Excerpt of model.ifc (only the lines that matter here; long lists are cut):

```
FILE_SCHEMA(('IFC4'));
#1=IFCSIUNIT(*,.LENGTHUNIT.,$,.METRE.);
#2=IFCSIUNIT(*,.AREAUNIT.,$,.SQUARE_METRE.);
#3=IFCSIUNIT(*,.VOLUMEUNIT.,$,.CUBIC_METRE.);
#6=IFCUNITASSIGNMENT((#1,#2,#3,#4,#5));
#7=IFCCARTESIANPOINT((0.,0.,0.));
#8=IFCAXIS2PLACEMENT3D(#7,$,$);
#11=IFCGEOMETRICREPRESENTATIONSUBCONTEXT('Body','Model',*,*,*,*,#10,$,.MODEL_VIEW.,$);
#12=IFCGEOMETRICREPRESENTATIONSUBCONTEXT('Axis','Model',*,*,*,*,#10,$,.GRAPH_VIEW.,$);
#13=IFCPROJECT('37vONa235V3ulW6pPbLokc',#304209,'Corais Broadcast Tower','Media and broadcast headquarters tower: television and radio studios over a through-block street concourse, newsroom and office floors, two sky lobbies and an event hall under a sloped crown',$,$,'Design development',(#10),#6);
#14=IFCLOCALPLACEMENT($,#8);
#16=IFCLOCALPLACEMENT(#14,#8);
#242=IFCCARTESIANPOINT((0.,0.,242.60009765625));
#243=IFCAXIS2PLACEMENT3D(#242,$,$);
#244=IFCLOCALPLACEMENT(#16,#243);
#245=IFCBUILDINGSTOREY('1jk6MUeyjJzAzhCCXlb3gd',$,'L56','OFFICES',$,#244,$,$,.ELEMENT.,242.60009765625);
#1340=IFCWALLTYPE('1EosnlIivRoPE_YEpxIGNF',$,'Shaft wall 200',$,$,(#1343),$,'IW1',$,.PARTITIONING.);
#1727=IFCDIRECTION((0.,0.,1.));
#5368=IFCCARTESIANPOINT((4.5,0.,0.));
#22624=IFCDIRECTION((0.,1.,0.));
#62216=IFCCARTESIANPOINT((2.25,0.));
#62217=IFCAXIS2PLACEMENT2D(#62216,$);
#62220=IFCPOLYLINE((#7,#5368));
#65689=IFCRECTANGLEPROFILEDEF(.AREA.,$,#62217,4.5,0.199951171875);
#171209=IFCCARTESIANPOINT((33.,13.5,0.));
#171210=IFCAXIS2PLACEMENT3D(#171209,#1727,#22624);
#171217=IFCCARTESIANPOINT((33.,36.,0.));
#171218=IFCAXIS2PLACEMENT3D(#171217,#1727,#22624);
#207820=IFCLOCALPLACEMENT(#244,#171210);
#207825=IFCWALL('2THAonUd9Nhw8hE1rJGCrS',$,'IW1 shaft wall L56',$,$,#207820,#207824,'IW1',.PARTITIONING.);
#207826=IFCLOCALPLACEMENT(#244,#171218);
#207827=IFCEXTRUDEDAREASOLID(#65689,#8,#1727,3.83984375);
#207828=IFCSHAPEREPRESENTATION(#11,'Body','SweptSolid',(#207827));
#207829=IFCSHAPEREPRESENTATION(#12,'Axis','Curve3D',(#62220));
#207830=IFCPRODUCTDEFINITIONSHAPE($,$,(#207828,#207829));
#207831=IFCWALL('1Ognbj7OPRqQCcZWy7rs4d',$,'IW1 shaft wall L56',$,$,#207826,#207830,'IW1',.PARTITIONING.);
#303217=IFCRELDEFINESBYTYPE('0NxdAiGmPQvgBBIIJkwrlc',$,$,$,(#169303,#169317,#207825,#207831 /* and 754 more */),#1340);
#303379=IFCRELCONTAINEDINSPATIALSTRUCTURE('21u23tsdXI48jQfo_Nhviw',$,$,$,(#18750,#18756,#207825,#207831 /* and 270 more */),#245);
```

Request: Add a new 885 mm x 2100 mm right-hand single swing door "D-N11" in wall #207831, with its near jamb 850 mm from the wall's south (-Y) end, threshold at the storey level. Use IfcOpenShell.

```python
import numpy as np
import ifcopenshell
import ifcopenshell.api.feature
import ifcopenshell.api.geometry
import ifcopenshell.api.root
import ifcopenshell.api.spatial
import ifcopenshell.geom
import ifcopenshell.util.element
import ifcopenshell.util.placement
import ifcopenshell.util.representation
import ifcopenshell.util.shape
import ifcopenshell.util.unit

model = ifcopenshell.open("model.ifc")
unit_scale = ifcopenshell.util.unit.calculate_unit_scale(model)
settings = ifcopenshell.geom.settings()


def volume(element):
    """Net volume in cubic metres, openings subtracted."""
    shape = ifcopenshell.geom.create_shape(settings, element)
    return ifcopenshell.util.shape.get_volume(shape.geometry)


wall = model.by_guid("1Ognbj7OPRqQCcZWy7rs4d")
storey = ifcopenshell.util.element.get_container(wall, ifc_class="IfcBuildingStorey")
context = ifcopenshell.util.representation.get_context(model, "Model", "Body", "MODEL_VIEW")
before = volume(wall)

width, height, from_end, sill = 0.885, 2.1, 0.85, 0.0  # metres

# The wall runs along its own X axis, and the end named is its -X end.
wall_shape = ifcopenshell.geom.create_shape(settings, wall)
x, y, z = ifcopenshell.util.shape.get_vertices(wall_shape.geometry).T
start = x.min() + from_end
face, thickness = float(y.min()), float(y.max() - y.min())
wall_matrix = ifcopenshell.util.placement.get_local_placement(wall.ObjectPlacement)
level = ifcopenshell.util.placement.get_local_placement(storey.ObjectPlacement)[2, 3]


def in_wall(x, y):
    """Placement at x, y metres in the wall's axes, at sill height."""
    matrix = wall_matrix.copy()
    matrix[:, 3] = wall_matrix @ np.array([x / unit_scale, y / unit_scale, 0.0, 1.0])
    matrix[2, 3] = level + sill / unit_scale
    return matrix


# Opening: a box that overshoots both wall faces by 50 mm.
opening = ifcopenshell.api.root.create_entity(model, ifc_class="IfcOpeningElement", predefined_type="OPENING")
box = ifcopenshell.api.geometry.add_wall_representation(
    model, context=context, length=width, height=height, thickness=thickness + 0.1
)
ifcopenshell.api.geometry.assign_representation(model, product=opening, representation=box)
ifcopenshell.api.geometry.edit_object_placement(model, product=opening, matrix=in_wall(start, face - 0.05), is_si=False)
ifcopenshell.api.feature.add_feature(model, feature=opening, element=wall)

door = ifcopenshell.api.root.create_entity(model, ifc_class="IfcDoor", name="D-N11", predefined_type="DOOR")
door.OverallWidth, door.OverallHeight = width / unit_scale, height / unit_scale
door.OperationType = "SINGLE_SWING_RIGHT"
body = ifcopenshell.api.geometry.add_door_representation(
    model,
    context=context,
    overall_width=door.OverallWidth,
    overall_height=door.OverallHeight,
    operation_type="SINGLE_SWING_RIGHT",
    lining_properties={"LiningDepth": thickness / unit_scale, "ThresholdDepth": thickness / unit_scale},
)
ifcopenshell.api.geometry.assign_representation(model, product=door, representation=body)
ifcopenshell.api.spatial.assign_container(model, products=[door], relating_structure=storey)
ifcopenshell.api.feature.add_filling(model, opening=opening, element=door)

# The lining spans the wall, so the door starts at the wall face.
ifcopenshell.api.geometry.edit_object_placement(model, product=door, matrix=in_wall(start, face), is_si=False)

after = volume(wall)

print(f"wall volume {before:.3f} -> {after:.3f} m3")

model.write("model_rev.ifc")
```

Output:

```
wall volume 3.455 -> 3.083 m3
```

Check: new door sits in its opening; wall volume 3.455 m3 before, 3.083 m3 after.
